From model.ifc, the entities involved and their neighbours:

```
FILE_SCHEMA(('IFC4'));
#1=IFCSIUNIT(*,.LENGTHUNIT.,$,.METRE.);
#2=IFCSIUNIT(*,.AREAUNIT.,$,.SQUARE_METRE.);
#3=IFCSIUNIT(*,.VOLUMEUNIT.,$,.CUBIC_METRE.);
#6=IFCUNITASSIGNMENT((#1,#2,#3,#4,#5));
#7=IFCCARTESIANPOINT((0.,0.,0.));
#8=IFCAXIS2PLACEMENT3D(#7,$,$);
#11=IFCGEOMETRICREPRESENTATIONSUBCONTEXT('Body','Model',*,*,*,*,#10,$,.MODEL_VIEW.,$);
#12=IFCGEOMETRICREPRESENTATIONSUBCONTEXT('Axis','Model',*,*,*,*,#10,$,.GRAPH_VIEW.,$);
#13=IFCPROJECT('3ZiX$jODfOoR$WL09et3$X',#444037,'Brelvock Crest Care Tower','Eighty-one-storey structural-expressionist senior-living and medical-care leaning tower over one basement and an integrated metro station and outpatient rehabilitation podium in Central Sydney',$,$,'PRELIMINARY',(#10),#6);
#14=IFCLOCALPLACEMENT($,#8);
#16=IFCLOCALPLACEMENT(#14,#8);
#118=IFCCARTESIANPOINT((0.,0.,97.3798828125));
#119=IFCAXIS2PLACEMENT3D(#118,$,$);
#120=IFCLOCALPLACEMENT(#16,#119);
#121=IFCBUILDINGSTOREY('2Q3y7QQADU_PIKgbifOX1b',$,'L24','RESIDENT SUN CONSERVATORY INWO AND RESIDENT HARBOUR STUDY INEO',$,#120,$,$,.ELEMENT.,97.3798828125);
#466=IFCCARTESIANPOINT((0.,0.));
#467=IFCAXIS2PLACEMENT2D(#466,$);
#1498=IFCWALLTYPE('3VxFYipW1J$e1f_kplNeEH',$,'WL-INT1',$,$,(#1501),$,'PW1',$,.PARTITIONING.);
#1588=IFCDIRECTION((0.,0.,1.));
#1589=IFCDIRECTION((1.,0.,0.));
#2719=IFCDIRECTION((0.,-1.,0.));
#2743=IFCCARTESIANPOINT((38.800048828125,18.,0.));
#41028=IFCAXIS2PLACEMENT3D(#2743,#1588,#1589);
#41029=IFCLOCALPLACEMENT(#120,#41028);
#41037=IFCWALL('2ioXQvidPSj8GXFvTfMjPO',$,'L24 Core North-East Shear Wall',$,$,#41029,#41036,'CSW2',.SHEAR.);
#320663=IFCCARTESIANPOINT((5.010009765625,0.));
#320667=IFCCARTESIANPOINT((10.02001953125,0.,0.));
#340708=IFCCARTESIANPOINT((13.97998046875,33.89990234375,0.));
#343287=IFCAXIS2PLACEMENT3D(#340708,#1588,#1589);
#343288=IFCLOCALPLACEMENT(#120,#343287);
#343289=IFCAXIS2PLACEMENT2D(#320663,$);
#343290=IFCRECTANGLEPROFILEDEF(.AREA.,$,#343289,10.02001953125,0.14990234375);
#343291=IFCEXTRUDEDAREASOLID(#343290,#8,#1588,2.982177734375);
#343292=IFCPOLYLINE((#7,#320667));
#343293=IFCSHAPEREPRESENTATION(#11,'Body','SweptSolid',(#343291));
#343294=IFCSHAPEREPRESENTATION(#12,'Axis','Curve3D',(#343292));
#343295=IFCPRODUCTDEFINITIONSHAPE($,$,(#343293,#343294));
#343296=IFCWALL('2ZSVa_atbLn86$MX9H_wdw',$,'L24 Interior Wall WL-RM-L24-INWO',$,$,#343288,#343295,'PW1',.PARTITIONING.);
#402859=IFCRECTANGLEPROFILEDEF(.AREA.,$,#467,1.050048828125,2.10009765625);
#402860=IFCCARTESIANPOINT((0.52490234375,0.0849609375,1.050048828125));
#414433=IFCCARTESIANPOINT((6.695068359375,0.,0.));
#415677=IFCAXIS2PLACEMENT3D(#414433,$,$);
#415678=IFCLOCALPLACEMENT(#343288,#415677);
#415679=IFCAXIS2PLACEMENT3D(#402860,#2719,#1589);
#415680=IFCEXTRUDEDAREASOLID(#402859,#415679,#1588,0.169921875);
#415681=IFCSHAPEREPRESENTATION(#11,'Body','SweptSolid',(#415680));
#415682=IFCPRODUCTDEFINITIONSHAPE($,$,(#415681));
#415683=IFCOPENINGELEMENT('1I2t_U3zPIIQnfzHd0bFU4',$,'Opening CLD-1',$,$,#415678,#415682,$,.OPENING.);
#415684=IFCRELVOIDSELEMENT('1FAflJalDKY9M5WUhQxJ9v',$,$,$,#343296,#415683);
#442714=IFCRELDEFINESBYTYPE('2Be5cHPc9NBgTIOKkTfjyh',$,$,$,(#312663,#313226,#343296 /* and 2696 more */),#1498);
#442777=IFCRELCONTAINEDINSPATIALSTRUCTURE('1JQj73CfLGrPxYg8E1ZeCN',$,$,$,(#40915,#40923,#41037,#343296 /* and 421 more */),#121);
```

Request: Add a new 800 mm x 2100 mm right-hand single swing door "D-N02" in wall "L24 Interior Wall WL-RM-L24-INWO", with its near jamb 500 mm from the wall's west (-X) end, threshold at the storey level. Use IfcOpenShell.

```python
import numpy as np
import ifcopenshell
import ifcopenshell.api.feature
import ifcopenshell.api.geometry
import ifcopenshell.api.root
import ifcopenshell.api.spatial
import ifcopenshell.geom
import ifcopenshell.util.element
import ifcopenshell.util.placement
import ifcopenshell.util.representation
import ifcopenshell.util.shape
import ifcopenshell.util.unit

model = ifcopenshell.open("model.ifc")
unit_scale = ifcopenshell.util.unit.calculate_unit_scale(model)
settings = ifcopenshell.geom.settings()


def volume(element):
    """Net volume in cubic metres, openings subtracted."""
    shape = ifcopenshell.geom.create_shape(settings, element)
    return ifcopenshell.util.shape.get_volume(shape.geometry)


wall = model.by_guid("2ZSVa_atbLn86$MX9H_wdw")
storey = ifcopenshell.util.element.get_container(wall, ifc_class="IfcBuildingStorey")
context = ifcopenshell.util.representation.get_context(model, "Model", "Body", "MODEL_VIEW")
before = volume(wall)

width, height, from_end, sill = 0.8, 2.1, 0.5, 0.0  # metres

# The wall runs along its own X axis, and the end named is its -X end.
wall_shape = ifcopenshell.geom.create_shape(settings, wall)
x, y, z = ifcopenshell.util.shape.get_vertices(wall_shape.geometry).T
start = x.min() + from_end
face, thickness = float(y.min()), float(y.max() - y.min())
wall_matrix = ifcopenshell.util.placement.get_local_placement(wall.ObjectPlacement)
level = ifcopenshell.util.placement.get_local_placement(storey.ObjectPlacement)[2, 3]


def in_wall(x, y):
    """Placement at x, y metres in the wall's axes, at sill height."""
    matrix = wall_matrix.copy()
    matrix[:, 3] = wall_matrix @ np.array([x / unit_scale, y / unit_scale, 0.0, 1.0])
    matrix[2, 3] = level + sill / unit_scale
    return matrix


# Opening: a box that overshoots both wall faces by 50 mm.
opening = ifcopenshell.api.root.create_entity(model, ifc_class="IfcOpeningElement", predefined_type="OPENING")
box = ifcopenshell.api.geometry.add_wall_representation(
    model, context=context, length=width, height=height, thickness=thickness + 0.1
)
ifcopenshell.api.geometry.assign_representation(model, product=opening, representation=box)
ifcopenshell.api.geometry.edit_object_placement(model, product=opening, matrix=in_wall(start, face - 0.05), is_si=False)
ifcopenshell.api.feature.add_feature(model, feature=opening, element=wall)

door = ifcopenshell.api.root.create_entity(model, ifc_class="IfcDoor", name="D-N02", predefined_type="DOOR")
door.OverallWidth, door.OverallHeight = width / unit_scale, height / unit_scale
door.OperationType = "SINGLE_SWING_RIGHT"
body = ifcopenshell.api.geometry.add_door_representation(
    model,
    context=context,
    overall_width=door.OverallWidth,
    overall_height=door.OverallHeight,
    operation_type="SINGLE_SWING_RIGHT",
    lining_properties={"LiningDepth": thickness / unit_scale, "ThresholdDepth": thickness / unit_scale},
)
ifcopenshell.api.geometry.assign_representation(model, product=door, representation=body)
ifcopenshell.api.spatial.assign_container(model, products=[door], relating_structure=storey)
ifcopenshell.api.feature.add_filling(model, opening=opening, element=door)

# The lining spans the wall, so the door starts at the wall face.
ifcopenshell.api.geometry.edit_object_placement(model, product=door, matrix=in_wall(start, face), is_si=False)

after = volume(wall)

print(f"wall volume {before:.3f} -> {after:.3f} m3")

model.write("model_updated.ifc")
```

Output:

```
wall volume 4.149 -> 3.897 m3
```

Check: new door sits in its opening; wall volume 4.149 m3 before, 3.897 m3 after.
